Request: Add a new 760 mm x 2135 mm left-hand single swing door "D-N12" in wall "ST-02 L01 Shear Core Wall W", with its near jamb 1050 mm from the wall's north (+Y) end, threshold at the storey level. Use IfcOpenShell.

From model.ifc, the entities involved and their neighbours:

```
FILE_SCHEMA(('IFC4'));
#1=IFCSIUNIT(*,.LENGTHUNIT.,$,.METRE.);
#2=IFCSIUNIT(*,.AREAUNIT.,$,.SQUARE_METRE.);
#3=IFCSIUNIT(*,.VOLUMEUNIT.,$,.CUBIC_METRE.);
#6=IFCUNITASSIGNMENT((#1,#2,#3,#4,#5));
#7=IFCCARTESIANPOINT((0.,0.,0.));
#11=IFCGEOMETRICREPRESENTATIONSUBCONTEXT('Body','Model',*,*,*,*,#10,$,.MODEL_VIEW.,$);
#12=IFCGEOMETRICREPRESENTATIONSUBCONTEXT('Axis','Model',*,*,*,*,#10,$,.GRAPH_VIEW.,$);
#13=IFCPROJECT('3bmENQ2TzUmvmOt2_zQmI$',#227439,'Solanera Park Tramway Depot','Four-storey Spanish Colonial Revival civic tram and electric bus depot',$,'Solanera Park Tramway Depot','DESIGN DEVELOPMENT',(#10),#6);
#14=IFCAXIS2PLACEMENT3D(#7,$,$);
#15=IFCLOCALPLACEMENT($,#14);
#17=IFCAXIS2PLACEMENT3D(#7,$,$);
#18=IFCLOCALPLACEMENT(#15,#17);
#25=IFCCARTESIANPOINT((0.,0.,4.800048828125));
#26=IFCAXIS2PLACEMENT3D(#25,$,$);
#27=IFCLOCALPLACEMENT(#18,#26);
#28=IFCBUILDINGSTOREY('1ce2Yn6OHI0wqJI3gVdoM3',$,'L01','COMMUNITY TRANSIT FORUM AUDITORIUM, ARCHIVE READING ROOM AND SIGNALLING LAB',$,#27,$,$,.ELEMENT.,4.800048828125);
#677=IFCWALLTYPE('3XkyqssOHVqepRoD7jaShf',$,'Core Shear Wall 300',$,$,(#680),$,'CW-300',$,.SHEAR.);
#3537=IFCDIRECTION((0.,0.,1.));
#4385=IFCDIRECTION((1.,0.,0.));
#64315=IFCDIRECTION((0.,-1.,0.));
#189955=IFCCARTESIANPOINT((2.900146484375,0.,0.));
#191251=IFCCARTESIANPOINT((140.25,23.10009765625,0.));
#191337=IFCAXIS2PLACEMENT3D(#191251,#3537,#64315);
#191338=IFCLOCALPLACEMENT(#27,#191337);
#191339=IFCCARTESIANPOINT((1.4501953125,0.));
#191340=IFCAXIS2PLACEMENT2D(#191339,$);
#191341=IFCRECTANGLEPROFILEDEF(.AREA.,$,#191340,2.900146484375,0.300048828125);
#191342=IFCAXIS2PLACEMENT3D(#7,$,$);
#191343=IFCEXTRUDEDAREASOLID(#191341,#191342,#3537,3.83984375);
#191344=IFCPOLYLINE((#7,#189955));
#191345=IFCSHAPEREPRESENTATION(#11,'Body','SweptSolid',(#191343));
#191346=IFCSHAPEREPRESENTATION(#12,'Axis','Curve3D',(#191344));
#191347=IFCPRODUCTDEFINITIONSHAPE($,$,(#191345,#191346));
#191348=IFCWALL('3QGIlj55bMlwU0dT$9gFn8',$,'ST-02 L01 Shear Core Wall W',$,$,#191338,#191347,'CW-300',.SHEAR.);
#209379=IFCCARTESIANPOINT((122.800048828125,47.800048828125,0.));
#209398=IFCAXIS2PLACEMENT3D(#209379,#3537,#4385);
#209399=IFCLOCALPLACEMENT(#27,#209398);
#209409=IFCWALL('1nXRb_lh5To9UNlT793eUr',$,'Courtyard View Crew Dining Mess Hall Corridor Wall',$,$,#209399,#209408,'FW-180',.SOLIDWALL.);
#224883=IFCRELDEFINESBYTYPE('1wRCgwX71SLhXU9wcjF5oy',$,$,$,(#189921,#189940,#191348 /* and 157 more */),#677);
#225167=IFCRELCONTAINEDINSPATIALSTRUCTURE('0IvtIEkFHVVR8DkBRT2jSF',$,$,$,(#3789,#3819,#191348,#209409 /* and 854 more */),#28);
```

```python
import numpy as np
import ifcopenshell
import ifcopenshell.api.feature
import ifcopenshell.api.geometry
import ifcopenshell.api.root
import ifcopenshell.api.spatial
import ifcopenshell.geom
import ifcopenshell.util.element
import ifcopenshell.util.placement
import ifcopenshell.util.representation
import ifcopenshell.util.shape
import ifcopenshell.util.unit

model = ifcopenshell.open("model.ifc")
unit_scale = ifcopenshell.util.unit.calculate_unit_scale(model)
settings = ifcopenshell.geom.settings()


def volume(element):
    """Net volume in cubic metres, openings subtracted."""
    shape = ifcopenshell.geom.create_shape(settings, element)
    return ifcopenshell.util.shape.get_volume(shape.geometry)


wall = model.by_guid("3QGIlj55bMlwU0dT$9gFn8")
storey = ifcopenshell.util.element.get_container(wall, ifc_class="IfcBuildingStorey")
context = ifcopenshell.util.representation.get_context(model, "Model", "Body", "MODEL_VIEW")
before = volume(wall)

width, height, from_end, sill = 0.76, 2.135, 1.05, 0.0  # metres

# The wall runs along its own X axis, and the end named is its -X end.
wall_shape = ifcopenshell.geom.create_shape(settings, wall)
x, y, z = ifcopenshell.util.shape.get_vertices(wall_shape.geometry).T
start = x.min() + from_end
face, thickness = float(y.min()), float(y.max() - y.min())
wall_matrix = ifcopenshell.util.placement.get_local_placement(wall.ObjectPlacement)
level = ifcopenshell.util.placement.get_local_placement(storey.ObjectPlacement)[2, 3]


def in_wall(x, y):
    """Placement at x, y metres in the wall's axes, at sill height."""
    matrix = wall_matrix.copy()
    matrix[:, 3] = wall_matrix @ np.array([x / unit_scale, y / unit_scale, 0.0, 1.0])
    matrix[2, 3] = level + sill / unit_scale
    return matrix


# Opening: a box that overshoots both wall faces by 50 mm.
opening = ifcopenshell.api.root.create_entity(model, ifc_class="IfcOpeningElement", predefined_type="OPENING")
box = ifcopenshell.api.geometry.add_wall_representation(
    model, context=context, length=width, height=height, thickness=thickness + 0.1
)
ifcopenshell.api.geometry.assign_representation(model, product=opening, representation=box)
ifcopenshell.api.geometry.edit_object_placement(model, product=opening, matrix=in_wall(start, face - 0.05), is_si=False)
ifcopenshell.api.feature.add_feature(model, feature=opening, element=wall)

door = ifcopenshell.api.root.create_entity(model, ifc_class="IfcDoor", name="D-N12", predefined_type="DOOR")
door.OverallWidth, door.OverallHeight = width / unit_scale, height / unit_scale
door.OperationType = "SINGLE_SWING_LEFT"
body = ifcopenshell.api.geometry.add_door_representation(
    model,
    context=context,
    overall_width=door.OverallWidth,
    overall_height=door.OverallHeight,
    operation_type="SINGLE_SWING_LEFT",
    lining_properties={"LiningDepth": thickness / unit_scale, "ThresholdDepth": thickness / unit_scale},
)
ifcopenshell.api.geometry.assign_representation(model, product=door, representation=body)
ifcopenshell.api.spatial.assign_container(model, products=[door], relating_structure=storey)
ifcopenshell.api.feature.add_filling(model, opening=opening, element=door)

# The lining spans the wall, so the door starts at the wall face.
ifcopenshell.api.geometry.edit_object_placement(model, product=door, matrix=in_wall(start, face), is_si=False)

after = volume(wall)

print(f"wall volume {before:.3f} -> {after:.3f} m3")

model.write("model_edited.ifc")
```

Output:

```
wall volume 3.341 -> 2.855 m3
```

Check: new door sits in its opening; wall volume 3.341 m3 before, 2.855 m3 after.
